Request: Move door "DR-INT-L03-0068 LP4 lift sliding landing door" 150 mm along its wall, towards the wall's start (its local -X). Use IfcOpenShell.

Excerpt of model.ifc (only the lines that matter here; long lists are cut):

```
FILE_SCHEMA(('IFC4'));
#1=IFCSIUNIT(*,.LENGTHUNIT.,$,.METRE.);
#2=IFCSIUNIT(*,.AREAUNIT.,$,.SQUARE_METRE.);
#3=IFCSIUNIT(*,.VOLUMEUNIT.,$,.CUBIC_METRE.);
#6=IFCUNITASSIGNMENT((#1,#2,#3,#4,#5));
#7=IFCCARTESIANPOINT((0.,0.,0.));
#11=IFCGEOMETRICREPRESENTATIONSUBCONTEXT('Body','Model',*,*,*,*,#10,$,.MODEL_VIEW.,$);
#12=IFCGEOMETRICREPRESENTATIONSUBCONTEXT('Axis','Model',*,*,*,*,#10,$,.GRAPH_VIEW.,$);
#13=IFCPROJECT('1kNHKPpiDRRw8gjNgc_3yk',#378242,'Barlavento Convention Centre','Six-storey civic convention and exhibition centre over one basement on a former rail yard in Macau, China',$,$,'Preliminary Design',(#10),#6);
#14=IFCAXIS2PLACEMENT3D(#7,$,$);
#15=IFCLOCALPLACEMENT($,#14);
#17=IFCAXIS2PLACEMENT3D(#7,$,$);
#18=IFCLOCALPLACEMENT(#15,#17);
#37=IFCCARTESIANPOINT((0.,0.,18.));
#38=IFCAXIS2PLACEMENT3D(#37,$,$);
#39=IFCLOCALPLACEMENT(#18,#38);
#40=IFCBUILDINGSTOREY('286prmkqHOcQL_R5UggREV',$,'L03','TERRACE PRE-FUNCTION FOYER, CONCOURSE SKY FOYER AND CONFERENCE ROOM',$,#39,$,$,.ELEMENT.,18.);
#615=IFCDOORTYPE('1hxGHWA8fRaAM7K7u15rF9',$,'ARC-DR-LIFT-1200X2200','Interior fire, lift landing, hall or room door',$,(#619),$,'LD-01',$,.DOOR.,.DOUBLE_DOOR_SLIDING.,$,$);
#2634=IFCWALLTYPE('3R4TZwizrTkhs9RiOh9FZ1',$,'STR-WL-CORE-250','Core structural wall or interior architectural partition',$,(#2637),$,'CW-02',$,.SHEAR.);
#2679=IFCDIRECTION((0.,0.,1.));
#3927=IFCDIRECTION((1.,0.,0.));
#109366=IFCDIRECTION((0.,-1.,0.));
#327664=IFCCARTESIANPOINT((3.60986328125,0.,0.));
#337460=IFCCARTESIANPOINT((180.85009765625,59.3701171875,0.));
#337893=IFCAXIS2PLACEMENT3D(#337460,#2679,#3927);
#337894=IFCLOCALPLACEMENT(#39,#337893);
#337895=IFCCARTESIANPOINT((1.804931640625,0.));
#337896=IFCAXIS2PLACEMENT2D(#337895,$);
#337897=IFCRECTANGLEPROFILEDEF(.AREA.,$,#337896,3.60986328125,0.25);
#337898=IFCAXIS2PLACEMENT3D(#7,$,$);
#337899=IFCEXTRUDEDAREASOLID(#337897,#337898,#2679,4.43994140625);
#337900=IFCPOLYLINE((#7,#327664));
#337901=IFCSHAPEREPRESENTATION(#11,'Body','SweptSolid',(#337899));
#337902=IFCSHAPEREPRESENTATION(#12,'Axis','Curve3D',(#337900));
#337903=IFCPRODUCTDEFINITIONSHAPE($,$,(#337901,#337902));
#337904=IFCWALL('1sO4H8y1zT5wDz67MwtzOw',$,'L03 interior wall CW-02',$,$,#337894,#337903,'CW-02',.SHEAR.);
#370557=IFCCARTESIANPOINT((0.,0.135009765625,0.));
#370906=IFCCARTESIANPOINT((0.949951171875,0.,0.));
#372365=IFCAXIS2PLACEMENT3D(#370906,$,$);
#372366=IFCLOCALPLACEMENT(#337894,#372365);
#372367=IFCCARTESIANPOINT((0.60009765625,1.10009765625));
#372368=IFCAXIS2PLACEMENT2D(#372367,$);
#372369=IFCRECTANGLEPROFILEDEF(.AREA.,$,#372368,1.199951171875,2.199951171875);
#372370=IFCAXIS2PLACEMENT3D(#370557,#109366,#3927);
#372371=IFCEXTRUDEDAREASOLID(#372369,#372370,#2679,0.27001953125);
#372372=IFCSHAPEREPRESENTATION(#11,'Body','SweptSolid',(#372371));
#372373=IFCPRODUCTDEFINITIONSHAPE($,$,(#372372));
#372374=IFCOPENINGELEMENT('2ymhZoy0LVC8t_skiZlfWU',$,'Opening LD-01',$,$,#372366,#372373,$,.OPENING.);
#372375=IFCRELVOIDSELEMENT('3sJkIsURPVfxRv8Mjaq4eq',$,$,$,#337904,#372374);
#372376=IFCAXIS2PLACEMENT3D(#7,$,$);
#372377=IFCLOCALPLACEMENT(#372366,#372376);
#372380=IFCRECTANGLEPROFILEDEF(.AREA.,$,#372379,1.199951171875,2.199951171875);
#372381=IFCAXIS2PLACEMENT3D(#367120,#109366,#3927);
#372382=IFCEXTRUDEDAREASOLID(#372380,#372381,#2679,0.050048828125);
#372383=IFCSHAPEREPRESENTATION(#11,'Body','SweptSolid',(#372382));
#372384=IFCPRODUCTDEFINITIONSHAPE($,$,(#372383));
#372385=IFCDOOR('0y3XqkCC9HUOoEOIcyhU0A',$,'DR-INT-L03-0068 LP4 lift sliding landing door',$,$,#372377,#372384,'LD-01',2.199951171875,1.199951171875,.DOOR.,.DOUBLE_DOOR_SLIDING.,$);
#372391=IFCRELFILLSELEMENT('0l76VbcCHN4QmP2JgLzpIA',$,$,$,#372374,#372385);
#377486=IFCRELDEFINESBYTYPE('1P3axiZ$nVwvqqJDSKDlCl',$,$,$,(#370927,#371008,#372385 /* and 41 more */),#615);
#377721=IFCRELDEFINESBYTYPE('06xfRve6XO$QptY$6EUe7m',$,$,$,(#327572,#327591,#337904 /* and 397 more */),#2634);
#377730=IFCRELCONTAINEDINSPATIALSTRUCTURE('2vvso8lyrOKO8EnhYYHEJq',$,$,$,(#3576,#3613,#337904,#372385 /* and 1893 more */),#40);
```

```python
import ifcopenshell
import ifcopenshell.api.geometry
import ifcopenshell.util.placement

model = ifcopenshell.open("model.ifc")

door = model.by_guid("0y3XqkCC9HUOoEOIcyhU0A")
opening = door.FillsVoids[0].RelatingOpeningElement
wall = opening.VoidsElements[0].RelatingBuildingElement

wall_matrix = ifcopenshell.util.placement.get_local_placement(wall.ObjectPlacement)
shift = wall_matrix[:3, 0] * -0.15
before = ifcopenshell.util.placement.get_local_placement(door.ObjectPlacement)[:3, 3].copy()

# The door is placed relative to its opening, so it follows when the opening moves.
matrix = ifcopenshell.util.placement.get_local_placement(opening.ObjectPlacement)
matrix[:3, 3] += shift
ifcopenshell.api.geometry.edit_object_placement(
    model, product=opening, matrix=matrix, is_si=False, should_transform_children=True
)

after = ifcopenshell.util.placement.get_local_placement(door.ObjectPlacement)[:3, 3]
print("door moved by", (after - before).round(3) + 0.0)

model.write("model_rev.ifc")
```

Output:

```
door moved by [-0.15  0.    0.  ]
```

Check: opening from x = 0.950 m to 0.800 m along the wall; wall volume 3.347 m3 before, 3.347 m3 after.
